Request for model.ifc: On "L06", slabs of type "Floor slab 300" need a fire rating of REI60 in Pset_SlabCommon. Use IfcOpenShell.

First a look at what the model holds.

```python
import ifcopenshell
import ifcopenshell.util.element

model = ifcopenshell.open("model.ifc")
print(model.schema)
storey = next(s for s in model.by_type("IfcBuildingStorey") if s.Name == "L06")
slabs = [e for e in ifcopenshell.util.element.get_decomposition(storey) if e.is_a("IfcSlab")]
seen = {}
for e in slabs:
    element_type = ifcopenshell.util.element.get_type(e)
    key = (element_type.Name if element_type != e and element_type else None, ifcopenshell.util.element.get_pset(e, "Pset_SlabCommon", "FireRating"))
    seen[key] = seen.get(key, 0) + 1
for (name, value), count in sorted(seen.items(), key=str):
    print(count, "x", name, "|", value)
```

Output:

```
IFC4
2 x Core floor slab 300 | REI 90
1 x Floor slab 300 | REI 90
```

```python
import ifcopenshell
import ifcopenshell.api.pset
import ifcopenshell.util.element

model = ifcopenshell.open("model.ifc")

storey = next(s for s in model.by_type("IfcBuildingStorey") if s.Name == "L06")
slabs = [e for e in ifcopenshell.util.element.get_decomposition(storey) if e.is_a("IfcSlab")]

count = 0
for e in slabs:
    element_type = ifcopenshell.util.element.get_type(e)
    if element_type in (None, e) or element_type.Name != "Floor slab 300":
        continue
    # add_pset returns the element's existing set when there is one.
    pset = ifcopenshell.api.pset.add_pset(model, product=e, name="Pset_SlabCommon")
    ifcopenshell.api.pset.edit_pset(model, pset=pset, properties={"FireRating": "REI60"})
    count += 1

print(count, "slabs updated")

model.write("model_rev.ifc")
```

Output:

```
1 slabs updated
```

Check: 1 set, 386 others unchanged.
